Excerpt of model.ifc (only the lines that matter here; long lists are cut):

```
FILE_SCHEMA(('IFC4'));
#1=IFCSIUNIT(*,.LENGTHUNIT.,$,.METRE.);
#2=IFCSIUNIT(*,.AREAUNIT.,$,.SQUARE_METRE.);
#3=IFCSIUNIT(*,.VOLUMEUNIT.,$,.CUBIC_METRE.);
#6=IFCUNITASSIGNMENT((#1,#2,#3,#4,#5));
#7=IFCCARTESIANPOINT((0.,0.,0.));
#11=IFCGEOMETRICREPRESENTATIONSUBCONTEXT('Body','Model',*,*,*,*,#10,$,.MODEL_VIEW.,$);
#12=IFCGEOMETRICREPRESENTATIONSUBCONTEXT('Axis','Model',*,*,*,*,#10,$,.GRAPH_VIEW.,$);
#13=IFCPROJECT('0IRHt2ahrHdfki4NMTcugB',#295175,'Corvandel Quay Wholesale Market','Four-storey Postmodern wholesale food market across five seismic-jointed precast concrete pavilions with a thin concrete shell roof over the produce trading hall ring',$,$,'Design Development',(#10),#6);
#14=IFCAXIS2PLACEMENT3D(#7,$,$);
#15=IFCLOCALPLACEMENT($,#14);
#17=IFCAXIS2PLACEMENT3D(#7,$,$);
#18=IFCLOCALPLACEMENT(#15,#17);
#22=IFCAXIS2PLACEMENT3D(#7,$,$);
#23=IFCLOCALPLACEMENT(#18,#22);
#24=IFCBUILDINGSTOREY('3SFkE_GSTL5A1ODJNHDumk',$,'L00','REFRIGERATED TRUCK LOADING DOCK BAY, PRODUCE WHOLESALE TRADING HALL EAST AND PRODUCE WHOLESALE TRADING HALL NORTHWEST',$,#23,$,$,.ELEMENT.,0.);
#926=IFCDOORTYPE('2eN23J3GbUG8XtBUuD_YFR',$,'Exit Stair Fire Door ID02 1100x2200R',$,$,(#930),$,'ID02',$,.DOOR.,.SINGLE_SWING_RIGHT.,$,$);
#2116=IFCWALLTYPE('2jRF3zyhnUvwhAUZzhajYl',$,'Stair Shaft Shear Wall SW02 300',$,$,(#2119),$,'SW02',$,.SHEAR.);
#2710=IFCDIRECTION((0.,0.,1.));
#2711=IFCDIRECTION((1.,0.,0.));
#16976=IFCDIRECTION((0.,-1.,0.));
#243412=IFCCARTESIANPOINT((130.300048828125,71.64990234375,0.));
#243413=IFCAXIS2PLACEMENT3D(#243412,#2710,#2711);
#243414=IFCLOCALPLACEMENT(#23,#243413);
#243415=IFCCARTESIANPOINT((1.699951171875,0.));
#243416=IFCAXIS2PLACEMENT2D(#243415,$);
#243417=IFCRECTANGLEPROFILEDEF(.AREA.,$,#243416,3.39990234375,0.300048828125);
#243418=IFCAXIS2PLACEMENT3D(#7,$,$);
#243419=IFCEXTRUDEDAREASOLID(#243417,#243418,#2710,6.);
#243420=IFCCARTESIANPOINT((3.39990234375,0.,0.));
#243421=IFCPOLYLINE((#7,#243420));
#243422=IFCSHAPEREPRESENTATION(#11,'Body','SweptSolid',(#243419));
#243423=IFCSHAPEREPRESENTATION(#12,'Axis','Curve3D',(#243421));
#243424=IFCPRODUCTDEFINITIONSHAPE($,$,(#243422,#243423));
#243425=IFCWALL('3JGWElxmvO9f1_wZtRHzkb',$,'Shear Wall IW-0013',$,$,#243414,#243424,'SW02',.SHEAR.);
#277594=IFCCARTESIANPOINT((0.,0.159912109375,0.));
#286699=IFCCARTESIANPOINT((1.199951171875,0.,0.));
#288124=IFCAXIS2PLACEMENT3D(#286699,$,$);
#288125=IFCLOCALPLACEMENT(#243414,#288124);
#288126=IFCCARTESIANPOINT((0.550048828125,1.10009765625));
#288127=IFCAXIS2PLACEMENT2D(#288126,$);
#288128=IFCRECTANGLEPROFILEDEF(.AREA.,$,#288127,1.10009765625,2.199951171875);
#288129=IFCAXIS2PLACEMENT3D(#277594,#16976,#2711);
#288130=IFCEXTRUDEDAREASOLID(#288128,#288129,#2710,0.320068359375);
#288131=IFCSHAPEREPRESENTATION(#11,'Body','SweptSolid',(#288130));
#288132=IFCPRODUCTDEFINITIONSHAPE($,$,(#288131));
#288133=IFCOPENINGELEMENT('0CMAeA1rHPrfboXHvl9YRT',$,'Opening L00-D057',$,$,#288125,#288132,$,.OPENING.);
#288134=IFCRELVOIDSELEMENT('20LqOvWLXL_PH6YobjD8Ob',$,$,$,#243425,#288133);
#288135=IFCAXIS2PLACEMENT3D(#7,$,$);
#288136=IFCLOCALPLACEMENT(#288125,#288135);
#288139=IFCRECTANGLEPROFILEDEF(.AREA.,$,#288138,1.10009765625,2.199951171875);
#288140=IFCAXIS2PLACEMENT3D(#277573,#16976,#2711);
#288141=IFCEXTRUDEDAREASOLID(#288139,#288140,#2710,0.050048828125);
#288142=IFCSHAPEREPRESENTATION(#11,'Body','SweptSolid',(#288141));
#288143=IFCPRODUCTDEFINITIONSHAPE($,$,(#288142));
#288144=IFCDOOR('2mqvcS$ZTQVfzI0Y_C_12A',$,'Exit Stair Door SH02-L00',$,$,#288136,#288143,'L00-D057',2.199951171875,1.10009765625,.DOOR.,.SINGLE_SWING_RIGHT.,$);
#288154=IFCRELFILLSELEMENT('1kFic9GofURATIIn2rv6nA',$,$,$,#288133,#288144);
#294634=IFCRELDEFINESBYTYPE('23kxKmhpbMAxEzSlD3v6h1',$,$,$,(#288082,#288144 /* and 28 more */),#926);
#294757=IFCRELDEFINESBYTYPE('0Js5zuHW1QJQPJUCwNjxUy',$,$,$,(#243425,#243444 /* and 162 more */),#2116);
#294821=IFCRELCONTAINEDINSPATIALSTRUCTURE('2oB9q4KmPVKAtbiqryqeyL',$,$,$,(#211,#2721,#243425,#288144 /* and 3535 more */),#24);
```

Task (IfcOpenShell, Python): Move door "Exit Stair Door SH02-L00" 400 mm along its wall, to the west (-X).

```python
import ifcopenshell
import ifcopenshell.api.geometry
import ifcopenshell.util.placement

model = ifcopenshell.open("model.ifc")

door = model.by_guid("2mqvcS$ZTQVfzI0Y_C_12A")
opening = door.FillsVoids[0].RelatingOpeningElement
wall = opening.VoidsElements[0].RelatingBuildingElement

wall_matrix = ifcopenshell.util.placement.get_local_placement(wall.ObjectPlacement)
shift = wall_matrix[:3, 0] * -0.4
before = ifcopenshell.util.placement.get_local_placement(door.ObjectPlacement)[:3, 3].copy()

# The door is placed relative to its opening, so it follows when the opening moves.
matrix = ifcopenshell.util.placement.get_local_placement(opening.ObjectPlacement)
matrix[:3, 3] += shift
ifcopenshell.api.geometry.edit_object_placement(
    model, product=opening, matrix=matrix, is_si=False, should_transform_children=True
)

after = ifcopenshell.util.placement.get_local_placement(door.ObjectPlacement)[:3, 3]
print("door moved by", (after - before).round(3) + 0.0)

model.write("model_v2.ifc")
```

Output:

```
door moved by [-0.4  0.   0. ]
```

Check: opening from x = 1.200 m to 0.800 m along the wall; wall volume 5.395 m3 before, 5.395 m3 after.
